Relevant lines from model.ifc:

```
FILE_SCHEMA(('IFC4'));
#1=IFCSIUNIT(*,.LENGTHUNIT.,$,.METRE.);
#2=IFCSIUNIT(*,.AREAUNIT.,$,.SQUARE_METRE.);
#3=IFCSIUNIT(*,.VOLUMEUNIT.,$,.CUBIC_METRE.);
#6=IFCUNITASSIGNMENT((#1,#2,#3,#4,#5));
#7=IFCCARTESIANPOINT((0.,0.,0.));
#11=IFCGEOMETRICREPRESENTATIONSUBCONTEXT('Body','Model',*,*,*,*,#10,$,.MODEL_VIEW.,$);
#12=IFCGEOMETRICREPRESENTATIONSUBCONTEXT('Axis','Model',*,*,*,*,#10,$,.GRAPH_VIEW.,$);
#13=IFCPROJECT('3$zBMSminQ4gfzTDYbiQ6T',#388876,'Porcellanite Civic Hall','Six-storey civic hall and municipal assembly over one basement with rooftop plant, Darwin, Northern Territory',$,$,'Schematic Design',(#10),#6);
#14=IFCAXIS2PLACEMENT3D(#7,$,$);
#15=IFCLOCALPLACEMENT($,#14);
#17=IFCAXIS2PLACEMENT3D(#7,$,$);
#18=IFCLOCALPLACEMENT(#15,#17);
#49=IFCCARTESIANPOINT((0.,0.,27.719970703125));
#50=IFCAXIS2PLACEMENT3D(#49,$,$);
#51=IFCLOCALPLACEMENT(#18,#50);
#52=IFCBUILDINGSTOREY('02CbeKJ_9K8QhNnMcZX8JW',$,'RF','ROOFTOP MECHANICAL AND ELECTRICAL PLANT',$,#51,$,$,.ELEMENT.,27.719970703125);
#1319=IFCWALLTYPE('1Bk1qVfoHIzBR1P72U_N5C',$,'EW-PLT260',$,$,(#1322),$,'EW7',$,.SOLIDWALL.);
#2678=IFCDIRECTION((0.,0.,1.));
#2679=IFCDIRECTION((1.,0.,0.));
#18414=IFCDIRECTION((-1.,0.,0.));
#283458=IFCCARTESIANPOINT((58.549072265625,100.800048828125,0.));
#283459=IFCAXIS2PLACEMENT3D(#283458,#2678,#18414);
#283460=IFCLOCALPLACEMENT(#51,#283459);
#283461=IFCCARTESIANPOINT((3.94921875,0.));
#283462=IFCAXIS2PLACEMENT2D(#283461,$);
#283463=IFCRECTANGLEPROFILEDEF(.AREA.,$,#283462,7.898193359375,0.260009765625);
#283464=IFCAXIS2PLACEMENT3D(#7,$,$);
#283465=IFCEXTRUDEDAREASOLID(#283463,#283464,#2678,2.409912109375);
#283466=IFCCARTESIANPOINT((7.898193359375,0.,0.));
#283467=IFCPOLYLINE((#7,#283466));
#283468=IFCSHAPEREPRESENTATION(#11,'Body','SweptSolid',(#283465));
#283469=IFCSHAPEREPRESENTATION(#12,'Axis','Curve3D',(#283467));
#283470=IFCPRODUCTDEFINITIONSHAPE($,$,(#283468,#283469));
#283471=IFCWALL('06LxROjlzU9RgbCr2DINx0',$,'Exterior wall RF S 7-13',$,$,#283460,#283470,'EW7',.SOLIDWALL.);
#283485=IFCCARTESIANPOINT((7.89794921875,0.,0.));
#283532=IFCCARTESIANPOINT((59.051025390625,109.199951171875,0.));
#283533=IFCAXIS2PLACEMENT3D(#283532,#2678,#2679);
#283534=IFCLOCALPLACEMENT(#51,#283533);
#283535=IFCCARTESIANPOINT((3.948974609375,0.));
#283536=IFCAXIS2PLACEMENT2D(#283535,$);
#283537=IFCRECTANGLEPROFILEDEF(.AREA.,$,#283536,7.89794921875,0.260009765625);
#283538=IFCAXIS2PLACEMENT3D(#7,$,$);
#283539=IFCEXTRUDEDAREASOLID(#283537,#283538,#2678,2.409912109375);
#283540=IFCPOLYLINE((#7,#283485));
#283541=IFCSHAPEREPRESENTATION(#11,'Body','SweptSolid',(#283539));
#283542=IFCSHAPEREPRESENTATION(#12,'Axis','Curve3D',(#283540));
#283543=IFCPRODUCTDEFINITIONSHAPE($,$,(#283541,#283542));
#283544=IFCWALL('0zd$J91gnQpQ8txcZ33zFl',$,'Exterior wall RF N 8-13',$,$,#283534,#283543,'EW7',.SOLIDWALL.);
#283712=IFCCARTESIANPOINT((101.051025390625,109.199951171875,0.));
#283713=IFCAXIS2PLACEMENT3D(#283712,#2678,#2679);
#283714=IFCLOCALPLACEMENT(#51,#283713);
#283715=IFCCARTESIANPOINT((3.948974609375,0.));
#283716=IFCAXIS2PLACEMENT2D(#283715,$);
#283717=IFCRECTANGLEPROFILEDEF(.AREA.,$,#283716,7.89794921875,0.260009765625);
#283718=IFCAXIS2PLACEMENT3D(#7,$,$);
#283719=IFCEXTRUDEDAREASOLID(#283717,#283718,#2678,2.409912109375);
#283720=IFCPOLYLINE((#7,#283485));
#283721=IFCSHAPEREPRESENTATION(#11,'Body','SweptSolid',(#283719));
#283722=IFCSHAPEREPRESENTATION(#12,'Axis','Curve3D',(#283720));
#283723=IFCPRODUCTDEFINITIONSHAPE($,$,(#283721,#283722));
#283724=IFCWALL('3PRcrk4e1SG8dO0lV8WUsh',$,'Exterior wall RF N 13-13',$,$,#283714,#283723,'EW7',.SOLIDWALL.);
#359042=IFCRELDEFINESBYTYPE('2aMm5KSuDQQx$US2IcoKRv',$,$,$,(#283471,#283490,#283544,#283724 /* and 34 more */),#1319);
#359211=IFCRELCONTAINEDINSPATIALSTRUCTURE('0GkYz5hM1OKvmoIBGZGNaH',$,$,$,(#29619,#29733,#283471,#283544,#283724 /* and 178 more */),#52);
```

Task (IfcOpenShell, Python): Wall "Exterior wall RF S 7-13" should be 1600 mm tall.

```python
import ifcopenshell
import ifcopenshell.geom
import ifcopenshell.util.representation
import ifcopenshell.util.shape
import ifcopenshell.util.unit

model = ifcopenshell.open("model.ifc")
unit_scale = ifcopenshell.util.unit.calculate_unit_scale(model)
settings = ifcopenshell.geom.settings()


def volume(element):
    """Net volume in cubic metres, openings subtracted."""
    shape = ifcopenshell.geom.create_shape(settings, element)
    return ifcopenshell.util.shape.get_volume(shape.geometry)


wall = model.by_guid("06LxROjlzU9RgbCr2DINx0")
before = volume(wall)

body = ifcopenshell.util.representation.get_representation(wall, "Model", "Body")
solid = body.Items[0]
old_height = solid.Depth
solid.Depth = 1.6 / unit_scale
after = volume(wall)

print(f"height {old_height:g} -> {solid.Depth:g}, volume {before:.3f} -> {after:.3f} m3")

model.write("model_edited.ifc")
```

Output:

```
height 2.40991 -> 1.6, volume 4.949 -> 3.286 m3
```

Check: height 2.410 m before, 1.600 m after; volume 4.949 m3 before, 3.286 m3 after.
